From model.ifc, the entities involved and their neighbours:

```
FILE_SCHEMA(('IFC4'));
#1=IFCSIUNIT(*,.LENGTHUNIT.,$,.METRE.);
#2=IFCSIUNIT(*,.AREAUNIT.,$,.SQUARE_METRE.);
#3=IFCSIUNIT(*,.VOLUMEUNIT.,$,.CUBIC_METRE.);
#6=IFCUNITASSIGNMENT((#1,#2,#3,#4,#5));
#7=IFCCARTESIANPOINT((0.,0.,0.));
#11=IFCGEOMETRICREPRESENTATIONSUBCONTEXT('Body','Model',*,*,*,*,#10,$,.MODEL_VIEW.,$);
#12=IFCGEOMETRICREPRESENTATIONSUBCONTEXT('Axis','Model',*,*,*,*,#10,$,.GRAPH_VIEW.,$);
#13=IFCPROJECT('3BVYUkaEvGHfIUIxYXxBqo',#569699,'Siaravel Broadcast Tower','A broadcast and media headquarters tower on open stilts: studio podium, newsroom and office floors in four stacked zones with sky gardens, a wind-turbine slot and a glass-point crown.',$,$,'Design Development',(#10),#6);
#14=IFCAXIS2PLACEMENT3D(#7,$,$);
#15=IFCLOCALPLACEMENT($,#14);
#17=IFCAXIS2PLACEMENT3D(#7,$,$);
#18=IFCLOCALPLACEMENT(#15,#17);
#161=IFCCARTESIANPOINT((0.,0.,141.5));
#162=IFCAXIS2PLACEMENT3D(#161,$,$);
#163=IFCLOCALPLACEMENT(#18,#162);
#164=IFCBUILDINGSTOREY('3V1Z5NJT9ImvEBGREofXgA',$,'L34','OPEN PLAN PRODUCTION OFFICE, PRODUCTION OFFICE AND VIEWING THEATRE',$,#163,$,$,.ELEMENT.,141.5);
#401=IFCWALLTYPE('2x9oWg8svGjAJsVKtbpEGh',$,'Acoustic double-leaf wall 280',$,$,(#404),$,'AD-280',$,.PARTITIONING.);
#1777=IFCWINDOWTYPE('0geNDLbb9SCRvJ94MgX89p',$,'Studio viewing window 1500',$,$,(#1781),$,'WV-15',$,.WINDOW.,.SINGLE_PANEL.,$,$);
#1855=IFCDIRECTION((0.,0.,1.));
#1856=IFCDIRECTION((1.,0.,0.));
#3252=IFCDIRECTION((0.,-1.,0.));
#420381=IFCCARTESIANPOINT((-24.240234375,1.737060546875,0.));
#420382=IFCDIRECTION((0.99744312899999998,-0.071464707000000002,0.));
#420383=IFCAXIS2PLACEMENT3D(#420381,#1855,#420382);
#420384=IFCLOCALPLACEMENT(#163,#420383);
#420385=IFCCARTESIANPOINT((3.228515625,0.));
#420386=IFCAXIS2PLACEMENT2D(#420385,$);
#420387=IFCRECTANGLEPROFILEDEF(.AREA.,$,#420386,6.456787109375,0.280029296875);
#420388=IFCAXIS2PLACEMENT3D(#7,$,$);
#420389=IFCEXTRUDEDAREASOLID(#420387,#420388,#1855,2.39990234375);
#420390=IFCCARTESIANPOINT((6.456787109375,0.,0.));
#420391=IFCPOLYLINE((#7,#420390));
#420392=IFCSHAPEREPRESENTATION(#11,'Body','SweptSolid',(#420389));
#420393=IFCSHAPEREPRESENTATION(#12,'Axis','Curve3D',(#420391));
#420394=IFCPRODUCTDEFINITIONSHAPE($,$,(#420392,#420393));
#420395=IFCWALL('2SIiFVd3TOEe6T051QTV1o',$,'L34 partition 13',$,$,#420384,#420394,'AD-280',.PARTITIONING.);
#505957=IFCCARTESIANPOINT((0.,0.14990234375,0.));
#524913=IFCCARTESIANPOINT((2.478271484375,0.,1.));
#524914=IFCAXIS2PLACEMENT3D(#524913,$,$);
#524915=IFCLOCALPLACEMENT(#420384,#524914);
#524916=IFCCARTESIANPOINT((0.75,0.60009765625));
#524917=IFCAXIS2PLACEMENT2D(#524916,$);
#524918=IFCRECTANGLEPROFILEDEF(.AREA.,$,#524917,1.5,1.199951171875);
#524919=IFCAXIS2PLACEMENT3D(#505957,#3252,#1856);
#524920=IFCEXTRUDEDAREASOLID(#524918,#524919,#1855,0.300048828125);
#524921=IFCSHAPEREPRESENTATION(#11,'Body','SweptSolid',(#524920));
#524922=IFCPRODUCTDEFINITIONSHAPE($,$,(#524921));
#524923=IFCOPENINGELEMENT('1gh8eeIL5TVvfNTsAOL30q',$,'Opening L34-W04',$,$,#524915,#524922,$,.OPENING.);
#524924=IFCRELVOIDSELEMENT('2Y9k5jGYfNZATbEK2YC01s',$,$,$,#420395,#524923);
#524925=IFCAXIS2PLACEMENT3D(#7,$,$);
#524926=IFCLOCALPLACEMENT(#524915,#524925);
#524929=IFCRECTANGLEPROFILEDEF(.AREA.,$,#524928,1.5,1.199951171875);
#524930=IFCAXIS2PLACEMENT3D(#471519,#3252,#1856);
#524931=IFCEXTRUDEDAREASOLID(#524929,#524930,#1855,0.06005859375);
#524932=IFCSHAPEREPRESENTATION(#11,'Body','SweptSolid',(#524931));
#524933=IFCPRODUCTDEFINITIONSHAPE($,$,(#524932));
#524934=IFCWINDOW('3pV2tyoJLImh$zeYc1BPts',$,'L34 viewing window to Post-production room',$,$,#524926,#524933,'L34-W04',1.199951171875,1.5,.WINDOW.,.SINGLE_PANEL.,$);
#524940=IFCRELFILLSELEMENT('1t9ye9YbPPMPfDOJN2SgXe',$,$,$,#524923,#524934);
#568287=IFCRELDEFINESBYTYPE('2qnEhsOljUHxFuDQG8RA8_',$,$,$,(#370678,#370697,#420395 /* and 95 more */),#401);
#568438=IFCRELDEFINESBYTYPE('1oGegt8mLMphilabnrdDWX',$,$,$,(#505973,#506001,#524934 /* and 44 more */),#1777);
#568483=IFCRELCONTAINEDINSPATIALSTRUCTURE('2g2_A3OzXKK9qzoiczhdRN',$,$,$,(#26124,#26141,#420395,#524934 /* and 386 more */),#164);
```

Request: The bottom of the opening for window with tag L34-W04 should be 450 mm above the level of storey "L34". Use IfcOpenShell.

```python
import numpy as np
import ifcopenshell
import ifcopenshell.api.geometry
import ifcopenshell.geom
import ifcopenshell.util.element
import ifcopenshell.util.placement
import ifcopenshell.util.shape
import ifcopenshell.util.unit

model = ifcopenshell.open("model.ifc")
unit_scale = ifcopenshell.util.unit.calculate_unit_scale(model)

window = model.by_guid("3pV2tyoJLImh$zeYc1BPts")
opening = window.FillsVoids[0].RelatingOpeningElement
storey = ifcopenshell.util.element.get_container(window, ifc_class="IfcBuildingStorey")
level = ifcopenshell.util.placement.get_local_placement(storey.ObjectPlacement)[2, 3]

# The opening's origin need not be at the sill, so measure its lowest point.
shape = ifcopenshell.geom.create_shape(ifcopenshell.geom.settings(), opening)
bottom = ifcopenshell.util.shape.get_shape_bottom_elevation(shape, shape.geometry) / unit_scale
dz = level + 0.45 - bottom

shift = np.array([0.0, 0.0, dz])
# The window is placed relative to its opening, so it follows when the opening moves.
matrix = ifcopenshell.util.placement.get_local_placement(opening.ObjectPlacement)
matrix[:3, 3] += shift
ifcopenshell.api.geometry.edit_object_placement(
    model, product=opening, matrix=matrix, is_si=False, should_transform_children=True
)

print(f"moved by {dz * unit_scale:+.3f} m")

model.write("model_updated.ifc")
```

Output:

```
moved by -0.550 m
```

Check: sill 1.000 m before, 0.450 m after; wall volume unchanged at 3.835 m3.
